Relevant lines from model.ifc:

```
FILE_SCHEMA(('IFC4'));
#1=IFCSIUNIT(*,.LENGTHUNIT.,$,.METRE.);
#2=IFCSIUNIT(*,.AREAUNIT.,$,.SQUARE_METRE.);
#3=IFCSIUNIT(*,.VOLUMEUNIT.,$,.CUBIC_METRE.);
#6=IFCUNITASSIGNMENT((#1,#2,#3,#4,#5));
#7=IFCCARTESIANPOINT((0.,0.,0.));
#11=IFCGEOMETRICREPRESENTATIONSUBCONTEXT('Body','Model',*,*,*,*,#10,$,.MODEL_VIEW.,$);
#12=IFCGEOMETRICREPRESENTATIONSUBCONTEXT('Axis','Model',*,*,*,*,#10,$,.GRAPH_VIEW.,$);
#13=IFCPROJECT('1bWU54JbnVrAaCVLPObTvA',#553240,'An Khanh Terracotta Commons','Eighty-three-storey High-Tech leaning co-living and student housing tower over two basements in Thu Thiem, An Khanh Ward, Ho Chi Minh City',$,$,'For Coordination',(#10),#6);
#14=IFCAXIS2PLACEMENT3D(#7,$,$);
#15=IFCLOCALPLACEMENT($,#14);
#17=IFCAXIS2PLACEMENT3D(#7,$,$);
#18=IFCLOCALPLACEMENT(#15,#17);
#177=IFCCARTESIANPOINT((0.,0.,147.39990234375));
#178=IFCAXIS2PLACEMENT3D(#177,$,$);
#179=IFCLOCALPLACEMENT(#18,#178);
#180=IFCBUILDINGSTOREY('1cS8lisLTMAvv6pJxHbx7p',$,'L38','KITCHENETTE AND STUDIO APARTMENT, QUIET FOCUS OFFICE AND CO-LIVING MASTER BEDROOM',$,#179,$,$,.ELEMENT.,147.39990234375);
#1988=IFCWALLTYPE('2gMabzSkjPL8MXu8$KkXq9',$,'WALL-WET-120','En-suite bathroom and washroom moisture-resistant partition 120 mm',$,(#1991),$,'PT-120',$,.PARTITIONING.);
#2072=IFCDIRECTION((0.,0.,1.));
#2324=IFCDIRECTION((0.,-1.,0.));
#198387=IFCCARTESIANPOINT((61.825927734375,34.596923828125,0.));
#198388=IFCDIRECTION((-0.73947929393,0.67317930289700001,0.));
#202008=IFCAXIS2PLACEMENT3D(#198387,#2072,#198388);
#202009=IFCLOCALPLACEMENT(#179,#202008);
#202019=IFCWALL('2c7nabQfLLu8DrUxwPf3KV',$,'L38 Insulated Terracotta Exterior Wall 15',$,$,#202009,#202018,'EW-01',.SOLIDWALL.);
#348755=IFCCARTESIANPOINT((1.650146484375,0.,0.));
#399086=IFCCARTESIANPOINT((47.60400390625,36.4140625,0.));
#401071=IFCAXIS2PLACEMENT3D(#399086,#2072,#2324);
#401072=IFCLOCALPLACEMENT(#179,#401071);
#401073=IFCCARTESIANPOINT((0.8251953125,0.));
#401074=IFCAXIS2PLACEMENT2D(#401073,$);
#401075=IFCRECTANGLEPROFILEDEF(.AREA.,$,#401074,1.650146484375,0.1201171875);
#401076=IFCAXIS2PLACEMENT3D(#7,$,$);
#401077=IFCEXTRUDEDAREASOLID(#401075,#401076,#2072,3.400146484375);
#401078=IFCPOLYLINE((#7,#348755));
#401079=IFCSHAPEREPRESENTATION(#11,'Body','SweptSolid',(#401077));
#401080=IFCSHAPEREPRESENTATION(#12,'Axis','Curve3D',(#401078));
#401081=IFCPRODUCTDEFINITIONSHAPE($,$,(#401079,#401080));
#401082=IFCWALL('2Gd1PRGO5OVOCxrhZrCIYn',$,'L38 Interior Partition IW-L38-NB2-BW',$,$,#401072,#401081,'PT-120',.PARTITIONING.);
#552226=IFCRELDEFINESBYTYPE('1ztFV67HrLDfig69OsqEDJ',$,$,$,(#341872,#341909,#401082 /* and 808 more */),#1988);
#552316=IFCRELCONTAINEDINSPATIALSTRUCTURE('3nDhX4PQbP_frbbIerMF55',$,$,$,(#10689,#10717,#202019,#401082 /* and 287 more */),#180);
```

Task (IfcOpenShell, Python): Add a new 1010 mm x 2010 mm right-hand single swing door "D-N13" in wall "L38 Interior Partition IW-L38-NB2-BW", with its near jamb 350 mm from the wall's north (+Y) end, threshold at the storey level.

```python
import numpy as np
import ifcopenshell
import ifcopenshell.api.feature
import ifcopenshell.api.geometry
import ifcopenshell.api.root
import ifcopenshell.api.spatial
import ifcopenshell.geom
import ifcopenshell.util.element
import ifcopenshell.util.placement
import ifcopenshell.util.representation
import ifcopenshell.util.shape
import ifcopenshell.util.unit

model = ifcopenshell.open("model.ifc")
unit_scale = ifcopenshell.util.unit.calculate_unit_scale(model)
settings = ifcopenshell.geom.settings()


def volume(element):
    """Net volume in cubic metres, openings subtracted."""
    shape = ifcopenshell.geom.create_shape(settings, element)
    return ifcopenshell.util.shape.get_volume(shape.geometry)


wall = model.by_guid("2Gd1PRGO5OVOCxrhZrCIYn")
storey = ifcopenshell.util.element.get_container(wall, ifc_class="IfcBuildingStorey")
context = ifcopenshell.util.representation.get_context(model, "Model", "Body", "MODEL_VIEW")
before = volume(wall)

width, height, from_end, sill = 1.01, 2.01, 0.35, 0.0  # metres

# The wall runs along its own X axis, and the end named is its -X end.
wall_shape = ifcopenshell.geom.create_shape(settings, wall)
x, y, z = ifcopenshell.util.shape.get_vertices(wall_shape.geometry).T
start = x.min() + from_end
face, thickness = float(y.min()), float(y.max() - y.min())
wall_matrix = ifcopenshell.util.placement.get_local_placement(wall.ObjectPlacement)
level = ifcopenshell.util.placement.get_local_placement(storey.ObjectPlacement)[2, 3]


def in_wall(x, y):
    """Placement at x, y metres in the wall's axes, at sill height."""
    matrix = wall_matrix.copy()
    matrix[:, 3] = wall_matrix @ np.array([x / unit_scale, y / unit_scale, 0.0, 1.0])
    matrix[2, 3] = level + sill / unit_scale
    return matrix


# Opening: a box that overshoots both wall faces by 50 mm.
opening = ifcopenshell.api.root.create_entity(model, ifc_class="IfcOpeningElement", predefined_type="OPENING")
box = ifcopenshell.api.geometry.add_wall_representation(
    model, context=context, length=width, height=height, thickness=thickness + 0.1
)
ifcopenshell.api.geometry.assign_representation(model, product=opening, representation=box)
ifcopenshell.api.geometry.edit_object_placement(model, product=opening, matrix=in_wall(start, face - 0.05), is_si=False)
ifcopenshell.api.feature.add_feature(model, feature=opening, element=wall)

door = ifcopenshell.api.root.create_entity(model, ifc_class="IfcDoor", name="D-N13", predefined_type="DOOR")
door.OverallWidth, door.OverallHeight = width / unit_scale, height / unit_scale
door.OperationType = "SINGLE_SWING_RIGHT"
body = ifcopenshell.api.geometry.add_door_representation(
    model,
    context=context,
    overall_width=door.OverallWidth,
    overall_height=door.OverallHeight,
    operation_type="SINGLE_SWING_RIGHT",
    lining_properties={"LiningDepth": thickness / unit_scale, "ThresholdDepth": thickness / unit_scale},
)
ifcopenshell.api.geometry.assign_representation(model, product=door, representation=body)
ifcopenshell.api.spatial.assign_container(model, products=[door], relating_structure=storey)
ifcopenshell.api.feature.add_filling(model, opening=opening, element=door)

# The lining spans the wall, so the door starts at the wall face.
ifcopenshell.api.geometry.edit_object_placement(model, product=door, matrix=in_wall(start, face), is_si=False)

after = volume(wall)

print(f"wall volume {before:.3f} -> {after:.3f} m3")

model.write("model_v2.ifc")
```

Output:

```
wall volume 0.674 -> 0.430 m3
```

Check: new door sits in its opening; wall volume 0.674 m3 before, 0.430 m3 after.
